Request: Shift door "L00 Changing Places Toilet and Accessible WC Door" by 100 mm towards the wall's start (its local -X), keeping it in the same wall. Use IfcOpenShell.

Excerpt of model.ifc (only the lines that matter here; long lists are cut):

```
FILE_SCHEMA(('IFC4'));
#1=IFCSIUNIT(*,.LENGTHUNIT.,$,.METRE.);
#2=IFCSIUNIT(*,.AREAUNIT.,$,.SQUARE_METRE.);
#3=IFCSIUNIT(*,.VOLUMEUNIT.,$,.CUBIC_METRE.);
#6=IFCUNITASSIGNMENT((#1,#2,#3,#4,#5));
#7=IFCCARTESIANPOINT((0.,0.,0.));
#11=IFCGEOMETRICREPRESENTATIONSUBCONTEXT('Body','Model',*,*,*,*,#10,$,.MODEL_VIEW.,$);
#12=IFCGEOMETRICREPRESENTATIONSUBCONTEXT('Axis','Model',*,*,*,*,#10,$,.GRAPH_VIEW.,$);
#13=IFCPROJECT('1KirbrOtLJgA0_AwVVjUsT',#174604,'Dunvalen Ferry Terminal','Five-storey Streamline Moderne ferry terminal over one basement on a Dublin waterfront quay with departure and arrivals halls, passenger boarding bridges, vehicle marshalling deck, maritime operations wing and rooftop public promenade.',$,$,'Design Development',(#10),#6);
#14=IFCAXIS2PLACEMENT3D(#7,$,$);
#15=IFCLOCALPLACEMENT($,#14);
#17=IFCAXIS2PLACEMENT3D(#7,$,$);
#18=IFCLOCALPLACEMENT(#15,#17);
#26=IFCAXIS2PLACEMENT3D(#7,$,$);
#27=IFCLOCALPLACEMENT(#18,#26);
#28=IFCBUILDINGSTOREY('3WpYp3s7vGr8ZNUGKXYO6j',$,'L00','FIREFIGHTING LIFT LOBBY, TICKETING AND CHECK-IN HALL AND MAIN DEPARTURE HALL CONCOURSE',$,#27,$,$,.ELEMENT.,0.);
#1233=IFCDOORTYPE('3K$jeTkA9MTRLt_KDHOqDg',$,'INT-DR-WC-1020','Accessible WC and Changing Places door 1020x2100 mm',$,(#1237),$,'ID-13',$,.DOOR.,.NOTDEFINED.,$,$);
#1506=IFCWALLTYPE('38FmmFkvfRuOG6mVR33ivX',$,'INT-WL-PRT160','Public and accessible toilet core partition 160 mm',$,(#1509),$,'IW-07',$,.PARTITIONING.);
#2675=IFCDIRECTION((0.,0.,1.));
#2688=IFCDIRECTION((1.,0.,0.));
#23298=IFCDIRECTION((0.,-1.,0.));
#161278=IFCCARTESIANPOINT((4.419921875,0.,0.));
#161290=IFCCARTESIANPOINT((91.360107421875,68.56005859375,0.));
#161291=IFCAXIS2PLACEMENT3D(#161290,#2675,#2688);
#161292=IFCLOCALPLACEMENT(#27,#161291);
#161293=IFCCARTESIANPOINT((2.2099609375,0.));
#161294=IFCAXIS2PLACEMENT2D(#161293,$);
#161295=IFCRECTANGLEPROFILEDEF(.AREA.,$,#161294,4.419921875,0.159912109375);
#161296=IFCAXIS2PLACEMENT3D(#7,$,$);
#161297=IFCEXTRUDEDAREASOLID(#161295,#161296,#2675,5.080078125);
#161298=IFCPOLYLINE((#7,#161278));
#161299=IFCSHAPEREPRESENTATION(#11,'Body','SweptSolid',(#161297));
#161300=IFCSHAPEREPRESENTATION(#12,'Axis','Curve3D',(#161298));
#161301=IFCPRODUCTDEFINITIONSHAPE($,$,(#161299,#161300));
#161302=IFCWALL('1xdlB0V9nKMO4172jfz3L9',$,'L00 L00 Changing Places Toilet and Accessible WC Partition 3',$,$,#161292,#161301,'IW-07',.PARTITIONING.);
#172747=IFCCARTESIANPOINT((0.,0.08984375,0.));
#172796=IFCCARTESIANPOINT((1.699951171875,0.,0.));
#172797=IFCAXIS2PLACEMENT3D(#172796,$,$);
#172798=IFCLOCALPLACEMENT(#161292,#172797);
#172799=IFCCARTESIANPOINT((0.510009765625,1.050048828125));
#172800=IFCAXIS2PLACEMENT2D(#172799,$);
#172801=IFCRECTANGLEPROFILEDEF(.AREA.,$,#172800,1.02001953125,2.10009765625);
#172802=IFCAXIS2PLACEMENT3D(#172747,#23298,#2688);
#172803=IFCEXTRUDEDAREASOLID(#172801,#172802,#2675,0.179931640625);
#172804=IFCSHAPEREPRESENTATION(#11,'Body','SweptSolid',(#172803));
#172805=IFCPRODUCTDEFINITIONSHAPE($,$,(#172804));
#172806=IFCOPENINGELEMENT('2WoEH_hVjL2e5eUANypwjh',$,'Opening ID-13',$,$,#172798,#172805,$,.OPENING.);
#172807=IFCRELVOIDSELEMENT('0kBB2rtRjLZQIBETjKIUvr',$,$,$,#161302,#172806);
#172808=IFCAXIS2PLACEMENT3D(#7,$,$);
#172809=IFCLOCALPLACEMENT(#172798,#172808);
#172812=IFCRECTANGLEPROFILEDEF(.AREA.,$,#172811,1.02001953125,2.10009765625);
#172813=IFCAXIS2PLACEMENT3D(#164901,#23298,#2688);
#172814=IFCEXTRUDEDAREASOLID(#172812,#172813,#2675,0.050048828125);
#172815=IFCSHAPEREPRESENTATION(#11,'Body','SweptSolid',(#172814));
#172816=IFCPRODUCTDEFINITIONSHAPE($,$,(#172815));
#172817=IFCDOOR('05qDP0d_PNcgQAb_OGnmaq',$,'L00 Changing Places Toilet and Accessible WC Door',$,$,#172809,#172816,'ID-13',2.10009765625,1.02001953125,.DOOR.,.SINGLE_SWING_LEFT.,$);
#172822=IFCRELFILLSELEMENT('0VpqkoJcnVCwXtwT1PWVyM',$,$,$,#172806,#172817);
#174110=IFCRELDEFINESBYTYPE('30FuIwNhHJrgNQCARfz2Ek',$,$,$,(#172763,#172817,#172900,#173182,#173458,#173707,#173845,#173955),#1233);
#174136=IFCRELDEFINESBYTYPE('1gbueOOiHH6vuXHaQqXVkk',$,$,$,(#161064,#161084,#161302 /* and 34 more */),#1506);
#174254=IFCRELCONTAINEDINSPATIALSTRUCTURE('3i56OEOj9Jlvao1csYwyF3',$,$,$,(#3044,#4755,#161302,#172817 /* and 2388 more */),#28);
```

```python
import ifcopenshell
import ifcopenshell.api.geometry
import ifcopenshell.util.placement
import ifcopenshell.util.unit

model = ifcopenshell.open("model.ifc")
unit_scale = ifcopenshell.util.unit.calculate_unit_scale(model)

door = model.by_guid("05qDP0d_PNcgQAb_OGnmaq")
opening = door.FillsVoids[0].RelatingOpeningElement
wall = opening.VoidsElements[0].RelatingBuildingElement

wall_matrix = ifcopenshell.util.placement.get_local_placement(wall.ObjectPlacement)
shift = wall_matrix[:3, 0] * -0.1 / unit_scale
before = ifcopenshell.util.placement.get_local_placement(door.ObjectPlacement)[:3, 3].copy()

# The door is placed relative to its opening, so it follows when the opening moves.
matrix = ifcopenshell.util.placement.get_local_placement(opening.ObjectPlacement)
matrix[:3, 3] += shift
ifcopenshell.api.geometry.edit_object_placement(
    model, product=opening, matrix=matrix, is_si=False, should_transform_children=True
)

after = ifcopenshell.util.placement.get_local_placement(door.ObjectPlacement)[:3, 3]
print("door moved by", (after - before).round(3) + 0.0)

model.write("model_v2.ifc")
```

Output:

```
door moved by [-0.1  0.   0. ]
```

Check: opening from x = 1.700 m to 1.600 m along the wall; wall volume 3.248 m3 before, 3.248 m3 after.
